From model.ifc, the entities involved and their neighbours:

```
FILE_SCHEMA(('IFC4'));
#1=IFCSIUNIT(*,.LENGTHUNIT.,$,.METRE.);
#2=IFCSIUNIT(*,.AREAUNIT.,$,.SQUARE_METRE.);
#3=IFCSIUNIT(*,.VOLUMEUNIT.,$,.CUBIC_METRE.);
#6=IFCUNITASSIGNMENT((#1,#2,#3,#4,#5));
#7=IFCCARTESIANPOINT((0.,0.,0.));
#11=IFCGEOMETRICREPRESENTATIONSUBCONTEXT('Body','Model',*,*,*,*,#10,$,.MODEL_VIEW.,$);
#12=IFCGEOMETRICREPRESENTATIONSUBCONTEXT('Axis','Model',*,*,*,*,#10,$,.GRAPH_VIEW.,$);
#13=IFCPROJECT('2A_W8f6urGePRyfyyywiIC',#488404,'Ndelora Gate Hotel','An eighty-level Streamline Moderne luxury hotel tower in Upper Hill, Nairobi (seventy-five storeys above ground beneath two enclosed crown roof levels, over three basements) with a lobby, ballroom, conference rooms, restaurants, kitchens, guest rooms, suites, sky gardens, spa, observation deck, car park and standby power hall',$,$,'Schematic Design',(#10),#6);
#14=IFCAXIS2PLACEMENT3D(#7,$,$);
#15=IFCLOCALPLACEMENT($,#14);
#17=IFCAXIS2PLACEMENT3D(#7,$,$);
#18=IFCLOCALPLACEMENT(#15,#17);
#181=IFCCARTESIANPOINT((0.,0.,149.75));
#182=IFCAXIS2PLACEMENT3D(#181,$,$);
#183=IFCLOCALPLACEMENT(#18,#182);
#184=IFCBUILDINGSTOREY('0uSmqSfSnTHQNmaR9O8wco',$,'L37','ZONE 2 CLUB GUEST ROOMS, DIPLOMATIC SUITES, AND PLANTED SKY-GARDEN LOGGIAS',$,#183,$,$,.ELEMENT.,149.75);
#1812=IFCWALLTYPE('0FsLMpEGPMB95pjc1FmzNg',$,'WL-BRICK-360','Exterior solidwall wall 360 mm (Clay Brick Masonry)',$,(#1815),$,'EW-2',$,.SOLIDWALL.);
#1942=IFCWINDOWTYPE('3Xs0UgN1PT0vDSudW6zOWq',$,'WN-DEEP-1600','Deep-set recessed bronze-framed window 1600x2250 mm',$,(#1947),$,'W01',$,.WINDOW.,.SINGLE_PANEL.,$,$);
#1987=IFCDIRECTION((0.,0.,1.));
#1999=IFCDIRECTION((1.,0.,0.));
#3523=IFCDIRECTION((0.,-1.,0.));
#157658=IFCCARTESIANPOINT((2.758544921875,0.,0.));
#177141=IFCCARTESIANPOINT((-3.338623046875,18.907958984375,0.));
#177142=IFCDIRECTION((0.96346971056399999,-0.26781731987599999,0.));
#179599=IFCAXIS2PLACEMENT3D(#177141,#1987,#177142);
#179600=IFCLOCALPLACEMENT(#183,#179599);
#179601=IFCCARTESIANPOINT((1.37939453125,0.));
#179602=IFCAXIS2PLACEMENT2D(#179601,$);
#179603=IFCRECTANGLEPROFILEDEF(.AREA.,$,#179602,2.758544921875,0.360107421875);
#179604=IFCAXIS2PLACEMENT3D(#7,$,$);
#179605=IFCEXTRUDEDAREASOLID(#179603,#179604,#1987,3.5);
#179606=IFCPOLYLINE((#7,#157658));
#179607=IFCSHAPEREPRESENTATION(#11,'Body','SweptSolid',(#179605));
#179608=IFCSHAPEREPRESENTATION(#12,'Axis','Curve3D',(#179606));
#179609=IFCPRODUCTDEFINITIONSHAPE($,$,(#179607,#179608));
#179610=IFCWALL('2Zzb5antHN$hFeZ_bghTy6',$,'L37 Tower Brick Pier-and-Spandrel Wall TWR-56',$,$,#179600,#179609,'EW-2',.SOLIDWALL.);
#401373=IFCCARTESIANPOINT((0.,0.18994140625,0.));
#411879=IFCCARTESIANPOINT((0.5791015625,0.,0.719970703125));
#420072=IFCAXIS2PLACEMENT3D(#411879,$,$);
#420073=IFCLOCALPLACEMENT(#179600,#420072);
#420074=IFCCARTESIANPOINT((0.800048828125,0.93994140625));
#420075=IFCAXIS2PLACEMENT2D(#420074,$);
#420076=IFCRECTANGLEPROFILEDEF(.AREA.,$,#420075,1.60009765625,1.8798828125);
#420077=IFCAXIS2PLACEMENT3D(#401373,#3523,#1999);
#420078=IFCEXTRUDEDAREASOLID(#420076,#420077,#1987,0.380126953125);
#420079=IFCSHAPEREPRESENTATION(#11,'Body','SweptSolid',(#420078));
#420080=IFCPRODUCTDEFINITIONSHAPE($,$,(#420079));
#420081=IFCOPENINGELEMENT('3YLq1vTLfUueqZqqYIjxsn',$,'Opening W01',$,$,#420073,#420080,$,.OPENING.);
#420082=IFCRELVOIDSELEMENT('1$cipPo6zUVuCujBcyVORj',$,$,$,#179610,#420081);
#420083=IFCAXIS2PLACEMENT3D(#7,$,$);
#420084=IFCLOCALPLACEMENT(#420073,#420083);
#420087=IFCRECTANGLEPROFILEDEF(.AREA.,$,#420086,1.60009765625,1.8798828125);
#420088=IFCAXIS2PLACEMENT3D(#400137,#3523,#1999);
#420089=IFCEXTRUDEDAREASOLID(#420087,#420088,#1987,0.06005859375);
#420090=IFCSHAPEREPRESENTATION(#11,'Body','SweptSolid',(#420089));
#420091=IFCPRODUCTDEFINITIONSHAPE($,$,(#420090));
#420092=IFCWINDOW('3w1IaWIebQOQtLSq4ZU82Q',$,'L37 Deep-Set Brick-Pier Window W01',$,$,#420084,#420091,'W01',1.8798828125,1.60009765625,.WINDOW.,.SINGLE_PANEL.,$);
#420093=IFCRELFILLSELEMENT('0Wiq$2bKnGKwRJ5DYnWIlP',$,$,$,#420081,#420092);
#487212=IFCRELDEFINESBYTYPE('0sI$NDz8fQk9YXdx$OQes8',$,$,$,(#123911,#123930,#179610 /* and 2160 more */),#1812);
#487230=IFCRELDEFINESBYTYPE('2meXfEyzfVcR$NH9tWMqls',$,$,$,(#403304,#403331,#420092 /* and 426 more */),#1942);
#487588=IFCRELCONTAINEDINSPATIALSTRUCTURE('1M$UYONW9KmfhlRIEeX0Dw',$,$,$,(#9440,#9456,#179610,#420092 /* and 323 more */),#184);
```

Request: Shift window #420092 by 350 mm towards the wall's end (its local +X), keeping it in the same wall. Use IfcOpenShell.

```python
import ifcopenshell
import ifcopenshell.api.geometry
import ifcopenshell.util.placement
import ifcopenshell.util.unit

model = ifcopenshell.open("model.ifc")
unit_scale = ifcopenshell.util.unit.calculate_unit_scale(model)

window = model.by_guid("3w1IaWIebQOQtLSq4ZU82Q")
opening = window.FillsVoids[0].RelatingOpeningElement
wall = opening.VoidsElements[0].RelatingBuildingElement

wall_matrix = ifcopenshell.util.placement.get_local_placement(wall.ObjectPlacement)
shift = wall_matrix[:3, 0] * 0.35 / unit_scale
before = ifcopenshell.util.placement.get_local_placement(window.ObjectPlacement)[:3, 3].copy()

# The window is placed relative to its opening, so it follows when the opening moves.
matrix = ifcopenshell.util.placement.get_local_placement(opening.ObjectPlacement)
matrix[:3, 3] += shift
ifcopenshell.api.geometry.edit_object_placement(
    model, product=opening, matrix=matrix, is_si=False, should_transform_children=True
)

after = ifcopenshell.util.placement.get_local_placement(window.ObjectPlacement)[:3, 3]
print("window moved by", (after - before).round(3) + 0.0)

model.write("model-out.ifc")
```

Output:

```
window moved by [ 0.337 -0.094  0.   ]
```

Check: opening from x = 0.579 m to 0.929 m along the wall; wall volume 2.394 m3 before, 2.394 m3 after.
